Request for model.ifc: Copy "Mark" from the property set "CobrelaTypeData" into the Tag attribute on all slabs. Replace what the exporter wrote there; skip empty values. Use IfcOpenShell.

First a look at what the model holds.

```python
import ifcopenshell
import ifcopenshell.util.element

model = ifcopenshell.open("model.ifc")
print(model.schema)
slabs = model.by_type("IfcSlab")
print(len(slabs), "slabs")
for e in slabs[:8]:
    source = ifcopenshell.util.element.get_pset(e, "CobrelaTypeData", "Mark")
    target = e.Tag
    print(e.id(), repr(source), repr(target), sep=" | ")
```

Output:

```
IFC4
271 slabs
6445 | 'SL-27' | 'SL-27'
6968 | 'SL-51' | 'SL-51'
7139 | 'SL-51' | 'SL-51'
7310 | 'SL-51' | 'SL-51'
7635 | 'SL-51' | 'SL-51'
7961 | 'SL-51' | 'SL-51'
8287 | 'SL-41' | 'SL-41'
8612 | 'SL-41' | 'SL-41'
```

```python
import ifcopenshell
import ifcopenshell.util.element

model = ifcopenshell.open("model.ifc")

count = 0
for e in model.by_type("IfcSlab"):
    value = ifcopenshell.util.element.get_pset(e, "CobrelaTypeData", "Mark")
    current = e.Tag
    if not value or not value.strip() or current == value:
        continue
    e.Tag = value
    count += 1

print(count, "slabs updated")

model.write("model_edited.ifc")
```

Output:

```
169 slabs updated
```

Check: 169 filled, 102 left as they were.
